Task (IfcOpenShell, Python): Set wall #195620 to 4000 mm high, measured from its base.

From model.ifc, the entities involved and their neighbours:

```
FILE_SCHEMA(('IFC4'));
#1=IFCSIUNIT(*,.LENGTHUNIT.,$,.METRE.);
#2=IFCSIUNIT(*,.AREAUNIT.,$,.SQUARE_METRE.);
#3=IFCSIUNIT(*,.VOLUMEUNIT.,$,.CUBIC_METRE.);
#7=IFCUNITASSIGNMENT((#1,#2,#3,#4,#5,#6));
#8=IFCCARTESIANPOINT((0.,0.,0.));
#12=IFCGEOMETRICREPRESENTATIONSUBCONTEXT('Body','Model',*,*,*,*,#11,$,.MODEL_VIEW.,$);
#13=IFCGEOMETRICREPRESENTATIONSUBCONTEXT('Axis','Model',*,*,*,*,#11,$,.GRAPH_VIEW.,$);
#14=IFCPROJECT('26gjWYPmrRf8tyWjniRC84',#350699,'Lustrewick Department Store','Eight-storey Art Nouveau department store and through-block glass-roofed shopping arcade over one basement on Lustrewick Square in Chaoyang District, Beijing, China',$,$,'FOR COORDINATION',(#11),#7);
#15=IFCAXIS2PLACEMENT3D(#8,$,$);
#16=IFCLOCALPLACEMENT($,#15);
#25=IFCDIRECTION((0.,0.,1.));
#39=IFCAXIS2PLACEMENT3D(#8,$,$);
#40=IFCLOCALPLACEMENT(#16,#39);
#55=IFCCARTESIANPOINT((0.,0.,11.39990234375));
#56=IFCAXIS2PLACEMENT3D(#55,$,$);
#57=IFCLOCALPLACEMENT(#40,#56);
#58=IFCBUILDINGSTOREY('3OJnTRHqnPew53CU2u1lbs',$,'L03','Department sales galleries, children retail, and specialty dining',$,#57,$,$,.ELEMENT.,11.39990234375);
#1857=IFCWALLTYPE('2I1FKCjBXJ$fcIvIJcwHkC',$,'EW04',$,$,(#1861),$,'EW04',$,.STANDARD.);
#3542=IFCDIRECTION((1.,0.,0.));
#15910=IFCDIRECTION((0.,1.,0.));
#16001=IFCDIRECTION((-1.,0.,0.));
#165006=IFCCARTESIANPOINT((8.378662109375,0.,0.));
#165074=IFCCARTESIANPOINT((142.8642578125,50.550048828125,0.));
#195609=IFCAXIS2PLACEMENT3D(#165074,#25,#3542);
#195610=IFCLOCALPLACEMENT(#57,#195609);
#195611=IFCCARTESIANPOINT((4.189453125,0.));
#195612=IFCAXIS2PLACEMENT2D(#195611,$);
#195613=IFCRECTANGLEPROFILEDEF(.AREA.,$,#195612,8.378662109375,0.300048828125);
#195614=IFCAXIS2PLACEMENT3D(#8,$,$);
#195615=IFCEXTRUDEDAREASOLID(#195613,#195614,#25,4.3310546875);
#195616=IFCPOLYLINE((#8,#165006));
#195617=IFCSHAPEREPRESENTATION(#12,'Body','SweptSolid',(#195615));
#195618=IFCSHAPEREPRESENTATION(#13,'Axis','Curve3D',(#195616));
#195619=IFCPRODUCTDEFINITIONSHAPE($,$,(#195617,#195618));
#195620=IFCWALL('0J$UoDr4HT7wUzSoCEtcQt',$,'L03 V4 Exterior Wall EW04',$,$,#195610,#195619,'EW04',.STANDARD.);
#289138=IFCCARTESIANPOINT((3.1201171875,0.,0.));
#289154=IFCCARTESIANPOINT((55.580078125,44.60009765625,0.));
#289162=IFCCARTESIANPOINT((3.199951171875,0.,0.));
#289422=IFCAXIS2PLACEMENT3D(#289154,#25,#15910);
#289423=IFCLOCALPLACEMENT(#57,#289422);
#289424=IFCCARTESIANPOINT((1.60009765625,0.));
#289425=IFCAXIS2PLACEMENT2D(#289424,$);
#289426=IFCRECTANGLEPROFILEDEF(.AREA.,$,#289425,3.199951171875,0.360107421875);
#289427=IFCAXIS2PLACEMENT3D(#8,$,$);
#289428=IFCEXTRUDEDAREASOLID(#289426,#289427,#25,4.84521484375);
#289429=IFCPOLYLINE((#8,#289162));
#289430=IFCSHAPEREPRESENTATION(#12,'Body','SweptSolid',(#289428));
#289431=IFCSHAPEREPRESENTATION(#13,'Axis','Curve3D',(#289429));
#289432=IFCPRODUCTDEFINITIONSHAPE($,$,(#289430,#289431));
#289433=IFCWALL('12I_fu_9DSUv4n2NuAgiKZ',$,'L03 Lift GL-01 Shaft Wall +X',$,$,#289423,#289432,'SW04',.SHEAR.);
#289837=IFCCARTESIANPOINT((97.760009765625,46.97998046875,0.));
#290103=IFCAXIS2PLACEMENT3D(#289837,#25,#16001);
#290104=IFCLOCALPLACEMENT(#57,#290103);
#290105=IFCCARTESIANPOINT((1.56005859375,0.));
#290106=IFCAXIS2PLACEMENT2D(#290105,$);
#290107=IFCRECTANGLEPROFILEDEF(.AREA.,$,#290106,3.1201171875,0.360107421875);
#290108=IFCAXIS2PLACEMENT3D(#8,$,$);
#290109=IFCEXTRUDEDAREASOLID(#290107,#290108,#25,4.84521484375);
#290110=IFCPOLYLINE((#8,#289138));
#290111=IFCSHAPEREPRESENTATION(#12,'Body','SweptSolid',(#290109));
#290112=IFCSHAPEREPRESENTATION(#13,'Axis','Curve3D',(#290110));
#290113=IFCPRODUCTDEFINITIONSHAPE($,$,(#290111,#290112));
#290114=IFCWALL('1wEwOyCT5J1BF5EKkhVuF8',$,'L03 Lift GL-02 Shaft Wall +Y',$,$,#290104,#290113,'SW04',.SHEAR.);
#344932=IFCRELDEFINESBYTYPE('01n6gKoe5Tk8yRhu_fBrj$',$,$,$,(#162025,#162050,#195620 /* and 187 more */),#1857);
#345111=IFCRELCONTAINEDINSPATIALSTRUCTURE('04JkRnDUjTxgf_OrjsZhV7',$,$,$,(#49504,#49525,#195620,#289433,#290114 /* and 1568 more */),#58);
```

```python
import ifcopenshell
import ifcopenshell.geom
import ifcopenshell.util.representation
import ifcopenshell.util.shape

model = ifcopenshell.open("model.ifc")
settings = ifcopenshell.geom.settings()


def volume(element):
    """Net volume in cubic metres, openings subtracted."""
    shape = ifcopenshell.geom.create_shape(settings, element)
    return ifcopenshell.util.shape.get_volume(shape.geometry)


wall = model.by_id(195620)
before = volume(wall)

body = ifcopenshell.util.representation.get_representation(wall, "Model", "Body")
solid = body.Items[0]
old_height = solid.Depth
solid.Depth = 4.0
after = volume(wall)

print(f"height {old_height:g} -> {solid.Depth:g}, volume {before:.3f} -> {after:.3f} m3")

model.write("model_updated.ifc")
```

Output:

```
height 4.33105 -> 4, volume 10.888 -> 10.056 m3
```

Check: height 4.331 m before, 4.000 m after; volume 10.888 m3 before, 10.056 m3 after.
